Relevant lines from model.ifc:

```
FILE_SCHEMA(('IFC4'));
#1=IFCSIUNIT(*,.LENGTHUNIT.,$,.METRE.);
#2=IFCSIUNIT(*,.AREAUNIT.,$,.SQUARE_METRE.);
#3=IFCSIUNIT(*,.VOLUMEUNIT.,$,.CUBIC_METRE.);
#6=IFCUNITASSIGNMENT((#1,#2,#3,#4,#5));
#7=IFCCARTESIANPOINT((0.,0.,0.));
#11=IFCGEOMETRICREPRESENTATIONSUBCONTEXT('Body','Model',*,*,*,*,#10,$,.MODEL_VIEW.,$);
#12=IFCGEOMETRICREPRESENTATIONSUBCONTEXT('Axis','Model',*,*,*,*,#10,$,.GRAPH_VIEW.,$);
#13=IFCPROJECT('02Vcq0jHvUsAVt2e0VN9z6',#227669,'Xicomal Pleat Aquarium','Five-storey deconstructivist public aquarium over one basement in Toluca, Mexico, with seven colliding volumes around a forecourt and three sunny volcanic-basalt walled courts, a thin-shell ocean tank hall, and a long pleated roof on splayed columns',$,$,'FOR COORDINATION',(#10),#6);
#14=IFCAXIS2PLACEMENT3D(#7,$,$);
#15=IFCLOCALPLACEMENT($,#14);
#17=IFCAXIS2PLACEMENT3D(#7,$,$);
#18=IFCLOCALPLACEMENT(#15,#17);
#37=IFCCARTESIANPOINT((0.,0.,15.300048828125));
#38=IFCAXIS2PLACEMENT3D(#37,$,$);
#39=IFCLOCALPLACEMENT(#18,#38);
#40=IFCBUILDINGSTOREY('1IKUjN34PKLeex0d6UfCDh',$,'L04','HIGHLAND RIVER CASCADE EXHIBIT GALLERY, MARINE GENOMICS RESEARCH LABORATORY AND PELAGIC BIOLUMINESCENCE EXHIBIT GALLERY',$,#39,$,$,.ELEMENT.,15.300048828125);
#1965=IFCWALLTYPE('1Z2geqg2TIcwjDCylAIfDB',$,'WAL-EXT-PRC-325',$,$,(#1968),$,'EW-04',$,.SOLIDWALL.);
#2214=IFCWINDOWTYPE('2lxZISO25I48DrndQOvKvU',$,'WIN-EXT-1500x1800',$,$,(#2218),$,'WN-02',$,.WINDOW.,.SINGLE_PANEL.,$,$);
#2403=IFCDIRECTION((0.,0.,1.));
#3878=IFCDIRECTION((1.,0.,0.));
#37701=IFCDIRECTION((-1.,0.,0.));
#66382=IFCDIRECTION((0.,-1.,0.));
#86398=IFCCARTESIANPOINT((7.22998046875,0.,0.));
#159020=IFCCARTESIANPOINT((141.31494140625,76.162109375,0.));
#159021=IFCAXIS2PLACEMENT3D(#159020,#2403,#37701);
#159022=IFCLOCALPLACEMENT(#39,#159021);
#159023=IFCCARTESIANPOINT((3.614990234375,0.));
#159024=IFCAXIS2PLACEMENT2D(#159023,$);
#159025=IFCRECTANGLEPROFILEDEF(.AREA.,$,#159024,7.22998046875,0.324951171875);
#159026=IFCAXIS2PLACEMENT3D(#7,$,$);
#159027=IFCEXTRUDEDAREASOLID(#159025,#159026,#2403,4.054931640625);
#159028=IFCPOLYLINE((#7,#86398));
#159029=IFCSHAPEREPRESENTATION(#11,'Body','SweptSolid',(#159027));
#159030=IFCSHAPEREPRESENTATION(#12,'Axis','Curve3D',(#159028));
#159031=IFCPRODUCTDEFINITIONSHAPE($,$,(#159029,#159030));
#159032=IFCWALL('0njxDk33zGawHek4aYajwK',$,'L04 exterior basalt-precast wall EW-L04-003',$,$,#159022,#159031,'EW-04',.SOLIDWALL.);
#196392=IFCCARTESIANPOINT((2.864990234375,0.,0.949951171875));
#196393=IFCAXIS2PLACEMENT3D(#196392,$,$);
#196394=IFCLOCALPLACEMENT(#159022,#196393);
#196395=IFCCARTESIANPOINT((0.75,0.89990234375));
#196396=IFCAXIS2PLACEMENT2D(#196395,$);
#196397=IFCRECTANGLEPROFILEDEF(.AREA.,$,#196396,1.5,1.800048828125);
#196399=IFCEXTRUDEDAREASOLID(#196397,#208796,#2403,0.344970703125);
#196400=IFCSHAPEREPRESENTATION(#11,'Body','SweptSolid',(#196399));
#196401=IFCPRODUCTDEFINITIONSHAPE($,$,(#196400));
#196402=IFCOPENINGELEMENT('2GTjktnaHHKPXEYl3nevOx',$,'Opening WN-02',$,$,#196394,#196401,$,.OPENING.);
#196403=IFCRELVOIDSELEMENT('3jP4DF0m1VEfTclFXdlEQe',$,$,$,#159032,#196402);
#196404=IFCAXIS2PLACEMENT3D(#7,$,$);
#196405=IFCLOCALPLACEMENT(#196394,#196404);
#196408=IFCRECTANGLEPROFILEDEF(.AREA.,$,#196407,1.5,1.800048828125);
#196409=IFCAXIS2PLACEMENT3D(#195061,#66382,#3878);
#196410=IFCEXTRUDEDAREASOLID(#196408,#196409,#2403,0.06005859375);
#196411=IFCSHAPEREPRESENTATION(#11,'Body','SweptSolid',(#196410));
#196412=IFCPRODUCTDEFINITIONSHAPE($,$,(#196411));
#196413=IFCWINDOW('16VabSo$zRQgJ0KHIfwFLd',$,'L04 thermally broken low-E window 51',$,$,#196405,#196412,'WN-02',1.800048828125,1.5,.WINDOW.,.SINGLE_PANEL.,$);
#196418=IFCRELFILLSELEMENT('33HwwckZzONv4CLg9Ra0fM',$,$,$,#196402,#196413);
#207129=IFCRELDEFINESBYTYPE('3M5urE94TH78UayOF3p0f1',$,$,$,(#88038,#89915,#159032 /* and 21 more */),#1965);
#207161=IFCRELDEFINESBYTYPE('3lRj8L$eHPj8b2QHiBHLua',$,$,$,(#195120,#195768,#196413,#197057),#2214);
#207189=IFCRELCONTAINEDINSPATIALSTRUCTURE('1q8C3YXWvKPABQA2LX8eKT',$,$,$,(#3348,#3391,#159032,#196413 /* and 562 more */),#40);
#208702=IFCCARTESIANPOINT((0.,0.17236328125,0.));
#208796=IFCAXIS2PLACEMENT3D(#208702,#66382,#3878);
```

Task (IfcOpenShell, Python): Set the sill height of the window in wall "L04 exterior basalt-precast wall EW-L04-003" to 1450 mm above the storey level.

```python
import numpy as np
import ifcopenshell
import ifcopenshell.api.geometry
import ifcopenshell.geom
import ifcopenshell.util.element
import ifcopenshell.util.placement
import ifcopenshell.util.shape
import ifcopenshell.util.unit

model = ifcopenshell.open("model.ifc")
unit_scale = ifcopenshell.util.unit.calculate_unit_scale(model)

window = model.by_guid("16VabSo$zRQgJ0KHIfwFLd")
opening = window.FillsVoids[0].RelatingOpeningElement
storey = ifcopenshell.util.element.get_container(window, ifc_class="IfcBuildingStorey")
level = ifcopenshell.util.placement.get_local_placement(storey.ObjectPlacement)[2, 3]

# The opening's origin need not be at the sill, so measure its lowest point.
shape = ifcopenshell.geom.create_shape(ifcopenshell.geom.settings(), opening)
bottom = ifcopenshell.util.shape.get_shape_bottom_elevation(shape, shape.geometry) / unit_scale
dz = level + 1.45 - bottom

shift = np.array([0.0, 0.0, dz])
# The window is placed relative to its opening, so it follows when the opening moves.
matrix = ifcopenshell.util.placement.get_local_placement(opening.ObjectPlacement)
matrix[:3, 3] += shift
ifcopenshell.api.geometry.edit_object_placement(
    model, product=opening, matrix=matrix, is_si=False, should_transform_children=True
)

print(f"moved by {dz * unit_scale:+.3f} m")

model.write("model-out.ifc")
```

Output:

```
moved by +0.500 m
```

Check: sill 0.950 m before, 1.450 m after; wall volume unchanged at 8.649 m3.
